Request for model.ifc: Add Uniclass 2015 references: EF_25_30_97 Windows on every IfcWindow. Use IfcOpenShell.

First a look at what the model holds.

```python
import ifcopenshell

model = ifcopenshell.open("model.ifc")
print(model.schema)
print("classifications:", [c.Name for c in model.by_type("IfcClassification")])
for ifc_class in ("IfcDoor", "IfcRoof", "IfcStair", "IfcWall", "IfcWindow"):
    print(ifc_class, len(model.by_type(ifc_class)))
```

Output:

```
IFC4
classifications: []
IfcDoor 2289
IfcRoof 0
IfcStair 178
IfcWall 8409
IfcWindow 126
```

```python
import ifcopenshell
import ifcopenshell.api.classification

model = ifcopenshell.open("model.ifc")

system = ifcopenshell.api.classification.add_classification(model, classification="Uniclass 2015")

codes = {
    "IfcWindow": ("EF_25_30_97", "Windows"),
}
for ifc_class, (code, name) in codes.items():
    products = model.by_type(ifc_class)
    ifcopenshell.api.classification.add_reference(
        model, products=products, classification=system, identification=code, name=name
    )
    print(code, len(products))

model.write("model_updated.ifc")
```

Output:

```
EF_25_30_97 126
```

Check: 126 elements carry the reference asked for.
